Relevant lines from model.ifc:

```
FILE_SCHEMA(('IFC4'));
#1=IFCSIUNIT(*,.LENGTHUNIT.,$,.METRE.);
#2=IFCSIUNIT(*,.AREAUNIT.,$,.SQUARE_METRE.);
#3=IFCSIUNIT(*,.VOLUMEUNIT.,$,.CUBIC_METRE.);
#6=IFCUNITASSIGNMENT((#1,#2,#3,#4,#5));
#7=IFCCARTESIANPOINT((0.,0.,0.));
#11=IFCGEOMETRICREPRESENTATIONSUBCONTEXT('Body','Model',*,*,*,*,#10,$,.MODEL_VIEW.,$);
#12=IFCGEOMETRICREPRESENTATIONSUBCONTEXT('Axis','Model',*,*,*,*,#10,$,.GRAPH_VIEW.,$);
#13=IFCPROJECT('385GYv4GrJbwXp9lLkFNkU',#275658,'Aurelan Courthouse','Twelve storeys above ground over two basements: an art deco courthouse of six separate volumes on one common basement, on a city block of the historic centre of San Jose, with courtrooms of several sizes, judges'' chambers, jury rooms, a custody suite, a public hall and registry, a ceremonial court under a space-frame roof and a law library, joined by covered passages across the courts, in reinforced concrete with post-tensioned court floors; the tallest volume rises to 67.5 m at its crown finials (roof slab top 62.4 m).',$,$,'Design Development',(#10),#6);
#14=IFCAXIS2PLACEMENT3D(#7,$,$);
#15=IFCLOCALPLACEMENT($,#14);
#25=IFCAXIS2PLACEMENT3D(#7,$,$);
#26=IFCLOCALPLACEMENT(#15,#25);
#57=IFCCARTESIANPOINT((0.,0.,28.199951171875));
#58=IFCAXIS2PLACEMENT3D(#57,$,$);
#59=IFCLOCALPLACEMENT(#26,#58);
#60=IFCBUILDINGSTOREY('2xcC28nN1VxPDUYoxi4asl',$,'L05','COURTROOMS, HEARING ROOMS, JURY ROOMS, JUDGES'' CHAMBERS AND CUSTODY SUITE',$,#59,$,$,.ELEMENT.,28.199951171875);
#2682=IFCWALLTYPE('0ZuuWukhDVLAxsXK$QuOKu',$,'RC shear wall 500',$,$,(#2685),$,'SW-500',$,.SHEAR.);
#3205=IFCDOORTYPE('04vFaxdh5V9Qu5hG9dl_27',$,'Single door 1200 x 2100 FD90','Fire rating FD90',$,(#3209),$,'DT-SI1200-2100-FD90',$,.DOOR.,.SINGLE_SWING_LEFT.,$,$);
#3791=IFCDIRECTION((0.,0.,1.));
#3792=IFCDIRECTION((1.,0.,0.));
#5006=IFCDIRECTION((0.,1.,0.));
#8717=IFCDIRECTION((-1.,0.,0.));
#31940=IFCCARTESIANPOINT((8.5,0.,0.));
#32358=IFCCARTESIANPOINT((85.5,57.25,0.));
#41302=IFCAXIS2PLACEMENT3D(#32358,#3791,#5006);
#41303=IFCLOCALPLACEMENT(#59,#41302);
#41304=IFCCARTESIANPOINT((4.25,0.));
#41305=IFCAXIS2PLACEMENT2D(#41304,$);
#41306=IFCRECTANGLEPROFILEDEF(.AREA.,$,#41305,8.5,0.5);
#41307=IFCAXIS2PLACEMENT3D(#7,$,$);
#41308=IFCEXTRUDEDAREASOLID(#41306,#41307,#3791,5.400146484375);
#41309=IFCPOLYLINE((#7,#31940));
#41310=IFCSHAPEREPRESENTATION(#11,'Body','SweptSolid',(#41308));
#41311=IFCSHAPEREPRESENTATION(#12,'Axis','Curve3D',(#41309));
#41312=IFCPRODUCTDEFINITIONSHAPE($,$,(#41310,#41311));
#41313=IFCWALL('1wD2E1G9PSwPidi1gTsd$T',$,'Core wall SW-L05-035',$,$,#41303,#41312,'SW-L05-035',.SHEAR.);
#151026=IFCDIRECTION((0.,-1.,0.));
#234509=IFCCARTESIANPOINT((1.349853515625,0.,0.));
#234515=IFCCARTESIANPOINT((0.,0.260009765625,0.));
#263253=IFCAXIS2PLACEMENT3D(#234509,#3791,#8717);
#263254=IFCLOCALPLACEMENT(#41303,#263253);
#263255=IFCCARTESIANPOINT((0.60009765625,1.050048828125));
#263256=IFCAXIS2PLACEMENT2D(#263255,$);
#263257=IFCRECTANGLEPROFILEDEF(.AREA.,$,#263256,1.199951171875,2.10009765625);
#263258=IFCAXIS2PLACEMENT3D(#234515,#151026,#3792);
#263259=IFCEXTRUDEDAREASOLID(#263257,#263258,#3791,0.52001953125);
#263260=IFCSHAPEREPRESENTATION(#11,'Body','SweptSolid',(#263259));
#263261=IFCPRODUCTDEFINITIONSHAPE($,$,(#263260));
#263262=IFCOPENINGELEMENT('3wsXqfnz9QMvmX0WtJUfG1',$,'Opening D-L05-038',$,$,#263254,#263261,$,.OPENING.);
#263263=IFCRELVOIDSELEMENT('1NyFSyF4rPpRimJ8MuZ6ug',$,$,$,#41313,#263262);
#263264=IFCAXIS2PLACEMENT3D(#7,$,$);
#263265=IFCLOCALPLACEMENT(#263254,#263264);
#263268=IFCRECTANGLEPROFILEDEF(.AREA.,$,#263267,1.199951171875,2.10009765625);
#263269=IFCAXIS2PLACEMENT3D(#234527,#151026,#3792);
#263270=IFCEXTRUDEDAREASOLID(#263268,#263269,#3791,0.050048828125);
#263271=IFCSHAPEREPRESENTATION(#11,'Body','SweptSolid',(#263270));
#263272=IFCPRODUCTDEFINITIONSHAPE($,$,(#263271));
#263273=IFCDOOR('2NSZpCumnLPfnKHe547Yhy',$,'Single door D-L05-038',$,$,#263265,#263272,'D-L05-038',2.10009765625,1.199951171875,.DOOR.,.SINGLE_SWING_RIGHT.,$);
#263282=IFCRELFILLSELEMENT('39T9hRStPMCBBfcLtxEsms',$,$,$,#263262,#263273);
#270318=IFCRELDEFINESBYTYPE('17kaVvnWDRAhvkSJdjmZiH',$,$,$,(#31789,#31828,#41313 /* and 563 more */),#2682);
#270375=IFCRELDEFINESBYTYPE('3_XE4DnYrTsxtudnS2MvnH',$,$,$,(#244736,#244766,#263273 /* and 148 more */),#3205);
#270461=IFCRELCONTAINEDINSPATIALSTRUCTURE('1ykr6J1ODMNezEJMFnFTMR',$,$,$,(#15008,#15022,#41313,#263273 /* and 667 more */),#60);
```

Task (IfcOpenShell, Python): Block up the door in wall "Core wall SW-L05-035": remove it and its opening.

```python
import ifcopenshell
import ifcopenshell.api.feature
import ifcopenshell.api.root
import ifcopenshell.geom
import ifcopenshell.util.shape

model = ifcopenshell.open("model.ifc")
settings = ifcopenshell.geom.settings()


def volume(element):
    """Net volume in cubic metres, openings subtracted."""
    shape = ifcopenshell.geom.create_shape(settings, element)
    return ifcopenshell.util.shape.get_volume(shape.geometry)


door = model.by_guid("2NSZpCumnLPfnKHe547Yhy")
opening = door.FillsVoids[0].RelatingOpeningElement
wall = opening.VoidsElements[0].RelatingBuildingElement
before = volume(wall)

ifcopenshell.api.root.remove_product(model, product=door)
ifcopenshell.api.feature.remove_feature(model, feature=opening)

after = volume(wall)

print(f"wall volume {before:.3f} -> {after:.3f} m3")

model.write("model-out.ifc")
```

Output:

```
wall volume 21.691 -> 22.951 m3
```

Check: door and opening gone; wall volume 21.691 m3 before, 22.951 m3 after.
